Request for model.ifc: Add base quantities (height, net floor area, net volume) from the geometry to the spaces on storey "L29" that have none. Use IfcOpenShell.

First a look at what the model holds.

```python
import ifcopenshell
import ifcopenshell.util.element
import ifcopenshell.util.unit

model = ifcopenshell.open("model.ifc")
print(model.schema)
for unit_type in ("LENGTHUNIT", "AREAUNIT", "VOLUMEUNIT"):
    print(unit_type, ifcopenshell.util.unit.calculate_unit_scale(model, unit_type))
storey = next(s for s in model.by_type("IfcBuildingStorey") if s.Name == "L29")
spaces = [e for e in ifcopenshell.util.element.get_decomposition(storey) if e.is_a("IfcSpace")]
for e in sorted(spaces, key=lambda e: e.id()):
    print(e.id(), e.is_a(), e.Name, list(ifcopenshell.util.element.get_psets(e, qtos_only=True)), sep=" | ")
```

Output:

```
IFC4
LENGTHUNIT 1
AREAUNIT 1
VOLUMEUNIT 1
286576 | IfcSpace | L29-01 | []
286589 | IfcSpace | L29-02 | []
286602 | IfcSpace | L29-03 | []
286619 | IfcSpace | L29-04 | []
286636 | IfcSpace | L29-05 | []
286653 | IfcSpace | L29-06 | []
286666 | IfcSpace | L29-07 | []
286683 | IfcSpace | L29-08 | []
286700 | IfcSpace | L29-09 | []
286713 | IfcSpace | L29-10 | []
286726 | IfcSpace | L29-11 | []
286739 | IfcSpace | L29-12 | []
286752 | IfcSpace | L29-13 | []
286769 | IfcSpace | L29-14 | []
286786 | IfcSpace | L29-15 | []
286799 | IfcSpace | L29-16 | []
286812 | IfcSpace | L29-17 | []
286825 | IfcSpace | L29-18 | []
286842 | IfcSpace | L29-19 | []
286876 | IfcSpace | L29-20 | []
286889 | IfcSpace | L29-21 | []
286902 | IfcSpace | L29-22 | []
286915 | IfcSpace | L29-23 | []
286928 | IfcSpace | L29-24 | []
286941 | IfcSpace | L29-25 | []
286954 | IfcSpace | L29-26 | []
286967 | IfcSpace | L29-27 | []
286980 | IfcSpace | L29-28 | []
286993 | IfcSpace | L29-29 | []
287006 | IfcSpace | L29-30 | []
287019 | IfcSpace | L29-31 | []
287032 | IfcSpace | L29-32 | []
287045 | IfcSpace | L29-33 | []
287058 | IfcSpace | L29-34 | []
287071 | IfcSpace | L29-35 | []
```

```python
import ifcopenshell
import ifcopenshell.api.pset
import ifcopenshell.geom
import ifcopenshell.util.element
import ifcopenshell.util.shape
import ifcopenshell.util.unit

model = ifcopenshell.open("model.ifc")
unit_scale = ifcopenshell.util.unit.calculate_unit_scale(model)
area_scale = ifcopenshell.util.unit.calculate_unit_scale(model, "AREAUNIT")
volume_scale = ifcopenshell.util.unit.calculate_unit_scale(model, "VOLUMEUNIT")
settings = ifcopenshell.geom.settings()

storey = next(s for s in model.by_type("IfcBuildingStorey") if s.Name == "L29")
spaces = [e for e in ifcopenshell.util.element.get_decomposition(storey) if e.is_a("IfcSpace")]

for e in sorted(spaces, key=lambda e: e.id()):
    if ifcopenshell.util.element.get_psets(e, qtos_only=True, should_inherit=False):
        continue
    # Geometry comes back in metres, in the element's own axes.
    shape = ifcopenshell.geom.create_shape(settings, e)
    values = {
        "Height": ifcopenshell.util.shape.get_z(shape.geometry) / unit_scale,
        "NetFloorArea": ifcopenshell.util.shape.get_footprint_area(shape.geometry) / area_scale,
        "NetVolume": ifcopenshell.util.shape.get_volume(shape.geometry) / volume_scale,
    }
    qto = ifcopenshell.api.pset.add_qto(model, product=e, name="Qto_SpaceBaseQuantities")
    ifcopenshell.api.pset.edit_qto(model, qto=qto, properties=values)
    print(e.id(), {k: round(v, 3) for k, v in values.items()})

model.write("model-out.ifc")
```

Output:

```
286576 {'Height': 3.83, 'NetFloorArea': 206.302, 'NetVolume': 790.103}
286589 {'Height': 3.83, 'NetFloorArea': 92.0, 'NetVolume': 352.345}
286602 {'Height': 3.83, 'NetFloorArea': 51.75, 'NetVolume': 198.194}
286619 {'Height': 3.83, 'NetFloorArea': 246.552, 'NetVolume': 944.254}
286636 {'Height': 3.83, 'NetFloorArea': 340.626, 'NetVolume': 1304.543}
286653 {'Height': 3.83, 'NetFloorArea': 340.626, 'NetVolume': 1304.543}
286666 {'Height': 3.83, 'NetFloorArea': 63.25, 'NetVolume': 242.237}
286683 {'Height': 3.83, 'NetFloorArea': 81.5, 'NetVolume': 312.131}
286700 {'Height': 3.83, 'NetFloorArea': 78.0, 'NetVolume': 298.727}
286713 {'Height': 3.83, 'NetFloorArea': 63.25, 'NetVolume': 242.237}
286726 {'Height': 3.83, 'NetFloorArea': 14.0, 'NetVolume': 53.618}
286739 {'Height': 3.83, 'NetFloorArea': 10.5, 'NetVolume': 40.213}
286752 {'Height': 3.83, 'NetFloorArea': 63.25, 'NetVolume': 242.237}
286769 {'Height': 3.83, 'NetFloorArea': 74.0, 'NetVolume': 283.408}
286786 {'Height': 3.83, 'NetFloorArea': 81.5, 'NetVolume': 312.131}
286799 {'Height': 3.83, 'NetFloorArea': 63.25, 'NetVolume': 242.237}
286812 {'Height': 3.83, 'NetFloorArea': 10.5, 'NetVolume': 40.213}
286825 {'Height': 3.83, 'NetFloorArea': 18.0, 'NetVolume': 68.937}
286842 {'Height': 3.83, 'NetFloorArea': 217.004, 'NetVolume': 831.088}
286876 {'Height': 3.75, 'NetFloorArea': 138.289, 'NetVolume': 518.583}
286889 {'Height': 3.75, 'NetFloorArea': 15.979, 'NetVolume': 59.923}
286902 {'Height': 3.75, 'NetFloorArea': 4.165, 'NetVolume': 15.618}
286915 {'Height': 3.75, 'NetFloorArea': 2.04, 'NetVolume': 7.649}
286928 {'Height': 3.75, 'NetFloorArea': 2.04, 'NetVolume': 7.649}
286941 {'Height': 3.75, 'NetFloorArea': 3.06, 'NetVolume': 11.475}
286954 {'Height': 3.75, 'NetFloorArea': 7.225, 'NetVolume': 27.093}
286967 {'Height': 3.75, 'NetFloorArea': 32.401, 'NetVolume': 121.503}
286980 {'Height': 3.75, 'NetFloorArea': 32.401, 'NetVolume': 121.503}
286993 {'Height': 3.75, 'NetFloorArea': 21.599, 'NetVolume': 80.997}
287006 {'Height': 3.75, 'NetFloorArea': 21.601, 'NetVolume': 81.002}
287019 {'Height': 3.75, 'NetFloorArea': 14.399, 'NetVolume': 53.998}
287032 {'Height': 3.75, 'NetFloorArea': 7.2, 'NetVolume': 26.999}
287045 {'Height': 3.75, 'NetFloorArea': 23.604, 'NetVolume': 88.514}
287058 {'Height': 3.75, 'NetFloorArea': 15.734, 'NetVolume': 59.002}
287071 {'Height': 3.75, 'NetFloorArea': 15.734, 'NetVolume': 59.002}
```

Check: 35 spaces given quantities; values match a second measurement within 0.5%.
